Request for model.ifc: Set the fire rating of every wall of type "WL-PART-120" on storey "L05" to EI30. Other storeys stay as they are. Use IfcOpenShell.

First a look at what the model holds.

```python
import ifcopenshell
import ifcopenshell.util.element

model = ifcopenshell.open("model.ifc")
print(model.schema)
storey = next(s for s in model.by_type("IfcBuildingStorey") if s.Name == "L05")
walls = [e for e in ifcopenshell.util.element.get_decomposition(storey) if e.is_a("IfcWall")]
seen = {}
for e in walls:
    element_type = ifcopenshell.util.element.get_type(e)
    key = (element_type.Name if element_type != e and element_type else None, ifcopenshell.util.element.get_pset(e, "Pset_WallCommon", "FireRating"))
    seen[key] = seen.get(key, 0) + 1
for (name, value), count in sorted(seen.items(), key=str):
    print(count, "x", name, "|", value)
```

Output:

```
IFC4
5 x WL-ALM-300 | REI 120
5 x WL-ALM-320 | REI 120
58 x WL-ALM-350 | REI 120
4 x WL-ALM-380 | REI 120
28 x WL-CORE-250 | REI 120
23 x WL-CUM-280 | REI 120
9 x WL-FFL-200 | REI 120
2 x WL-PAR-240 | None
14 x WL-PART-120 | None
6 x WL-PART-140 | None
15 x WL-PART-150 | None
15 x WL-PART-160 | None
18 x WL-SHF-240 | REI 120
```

```python
import ifcopenshell
import ifcopenshell.api.pset
import ifcopenshell.util.element

model = ifcopenshell.open("model.ifc")

storey = next(s for s in model.by_type("IfcBuildingStorey") if s.Name == "L05")
walls = [e for e in ifcopenshell.util.element.get_decomposition(storey) if e.is_a("IfcWall")]

count = 0
for e in walls:
    element_type = ifcopenshell.util.element.get_type(e)
    if element_type in (None, e) or element_type.Name != "WL-PART-120":
        continue
    # add_pset returns the element's existing set when there is one.
    pset = ifcopenshell.api.pset.add_pset(model, product=e, name="Pset_WallCommon")
    ifcopenshell.api.pset.edit_pset(model, pset=pset, properties={"FireRating": "EI30"})
    count += 1

print(count, "walls updated")

model.write("model_rev.ifc")
```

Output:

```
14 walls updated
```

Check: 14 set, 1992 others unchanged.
